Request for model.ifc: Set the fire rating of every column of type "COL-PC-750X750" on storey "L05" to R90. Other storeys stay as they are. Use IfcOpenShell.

First a look at what the model holds.

```python
import ifcopenshell
import ifcopenshell.util.element

model = ifcopenshell.open("model.ifc")
print(model.schema)
storey = next(s for s in model.by_type("IfcBuildingStorey") if s.Name == "L05")
columns = [e for e in ifcopenshell.util.element.get_decomposition(storey) if e.is_a("IfcColumn")]
seen = {}
for e in columns:
    element_type = ifcopenshell.util.element.get_type(e)
    key = (element_type.Name if element_type != e and element_type else None, ifcopenshell.util.element.get_pset(e, "Pset_ColumnCommon", "FireRating"))
    seen[key] = seen.get(key, 0) + 1
for (name, value), count in sorted(seen.items(), key=str):
    print(count, "x", name, "|", value)
```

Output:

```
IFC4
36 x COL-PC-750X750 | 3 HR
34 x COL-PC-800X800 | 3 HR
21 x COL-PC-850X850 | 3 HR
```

```python
import ifcopenshell
import ifcopenshell.api.pset
import ifcopenshell.util.element

model = ifcopenshell.open("model.ifc")

storey = next(s for s in model.by_type("IfcBuildingStorey") if s.Name == "L05")
columns = [e for e in ifcopenshell.util.element.get_decomposition(storey) if e.is_a("IfcColumn")]

count = 0
for e in columns:
    element_type = ifcopenshell.util.element.get_type(e)
    if element_type in (None, e) or element_type.Name != "COL-PC-750X750":
        continue
    # add_pset returns the element's existing set when there is one.
    pset = ifcopenshell.api.pset.add_pset(model, product=e, name="Pset_ColumnCommon")
    ifcopenshell.api.pset.edit_pset(model, pset=pset, properties={"FireRating": "R90"})
    count += 1

print(count, "columns updated")

model.write("model-out.ifc")
```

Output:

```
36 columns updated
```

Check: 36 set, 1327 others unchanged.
